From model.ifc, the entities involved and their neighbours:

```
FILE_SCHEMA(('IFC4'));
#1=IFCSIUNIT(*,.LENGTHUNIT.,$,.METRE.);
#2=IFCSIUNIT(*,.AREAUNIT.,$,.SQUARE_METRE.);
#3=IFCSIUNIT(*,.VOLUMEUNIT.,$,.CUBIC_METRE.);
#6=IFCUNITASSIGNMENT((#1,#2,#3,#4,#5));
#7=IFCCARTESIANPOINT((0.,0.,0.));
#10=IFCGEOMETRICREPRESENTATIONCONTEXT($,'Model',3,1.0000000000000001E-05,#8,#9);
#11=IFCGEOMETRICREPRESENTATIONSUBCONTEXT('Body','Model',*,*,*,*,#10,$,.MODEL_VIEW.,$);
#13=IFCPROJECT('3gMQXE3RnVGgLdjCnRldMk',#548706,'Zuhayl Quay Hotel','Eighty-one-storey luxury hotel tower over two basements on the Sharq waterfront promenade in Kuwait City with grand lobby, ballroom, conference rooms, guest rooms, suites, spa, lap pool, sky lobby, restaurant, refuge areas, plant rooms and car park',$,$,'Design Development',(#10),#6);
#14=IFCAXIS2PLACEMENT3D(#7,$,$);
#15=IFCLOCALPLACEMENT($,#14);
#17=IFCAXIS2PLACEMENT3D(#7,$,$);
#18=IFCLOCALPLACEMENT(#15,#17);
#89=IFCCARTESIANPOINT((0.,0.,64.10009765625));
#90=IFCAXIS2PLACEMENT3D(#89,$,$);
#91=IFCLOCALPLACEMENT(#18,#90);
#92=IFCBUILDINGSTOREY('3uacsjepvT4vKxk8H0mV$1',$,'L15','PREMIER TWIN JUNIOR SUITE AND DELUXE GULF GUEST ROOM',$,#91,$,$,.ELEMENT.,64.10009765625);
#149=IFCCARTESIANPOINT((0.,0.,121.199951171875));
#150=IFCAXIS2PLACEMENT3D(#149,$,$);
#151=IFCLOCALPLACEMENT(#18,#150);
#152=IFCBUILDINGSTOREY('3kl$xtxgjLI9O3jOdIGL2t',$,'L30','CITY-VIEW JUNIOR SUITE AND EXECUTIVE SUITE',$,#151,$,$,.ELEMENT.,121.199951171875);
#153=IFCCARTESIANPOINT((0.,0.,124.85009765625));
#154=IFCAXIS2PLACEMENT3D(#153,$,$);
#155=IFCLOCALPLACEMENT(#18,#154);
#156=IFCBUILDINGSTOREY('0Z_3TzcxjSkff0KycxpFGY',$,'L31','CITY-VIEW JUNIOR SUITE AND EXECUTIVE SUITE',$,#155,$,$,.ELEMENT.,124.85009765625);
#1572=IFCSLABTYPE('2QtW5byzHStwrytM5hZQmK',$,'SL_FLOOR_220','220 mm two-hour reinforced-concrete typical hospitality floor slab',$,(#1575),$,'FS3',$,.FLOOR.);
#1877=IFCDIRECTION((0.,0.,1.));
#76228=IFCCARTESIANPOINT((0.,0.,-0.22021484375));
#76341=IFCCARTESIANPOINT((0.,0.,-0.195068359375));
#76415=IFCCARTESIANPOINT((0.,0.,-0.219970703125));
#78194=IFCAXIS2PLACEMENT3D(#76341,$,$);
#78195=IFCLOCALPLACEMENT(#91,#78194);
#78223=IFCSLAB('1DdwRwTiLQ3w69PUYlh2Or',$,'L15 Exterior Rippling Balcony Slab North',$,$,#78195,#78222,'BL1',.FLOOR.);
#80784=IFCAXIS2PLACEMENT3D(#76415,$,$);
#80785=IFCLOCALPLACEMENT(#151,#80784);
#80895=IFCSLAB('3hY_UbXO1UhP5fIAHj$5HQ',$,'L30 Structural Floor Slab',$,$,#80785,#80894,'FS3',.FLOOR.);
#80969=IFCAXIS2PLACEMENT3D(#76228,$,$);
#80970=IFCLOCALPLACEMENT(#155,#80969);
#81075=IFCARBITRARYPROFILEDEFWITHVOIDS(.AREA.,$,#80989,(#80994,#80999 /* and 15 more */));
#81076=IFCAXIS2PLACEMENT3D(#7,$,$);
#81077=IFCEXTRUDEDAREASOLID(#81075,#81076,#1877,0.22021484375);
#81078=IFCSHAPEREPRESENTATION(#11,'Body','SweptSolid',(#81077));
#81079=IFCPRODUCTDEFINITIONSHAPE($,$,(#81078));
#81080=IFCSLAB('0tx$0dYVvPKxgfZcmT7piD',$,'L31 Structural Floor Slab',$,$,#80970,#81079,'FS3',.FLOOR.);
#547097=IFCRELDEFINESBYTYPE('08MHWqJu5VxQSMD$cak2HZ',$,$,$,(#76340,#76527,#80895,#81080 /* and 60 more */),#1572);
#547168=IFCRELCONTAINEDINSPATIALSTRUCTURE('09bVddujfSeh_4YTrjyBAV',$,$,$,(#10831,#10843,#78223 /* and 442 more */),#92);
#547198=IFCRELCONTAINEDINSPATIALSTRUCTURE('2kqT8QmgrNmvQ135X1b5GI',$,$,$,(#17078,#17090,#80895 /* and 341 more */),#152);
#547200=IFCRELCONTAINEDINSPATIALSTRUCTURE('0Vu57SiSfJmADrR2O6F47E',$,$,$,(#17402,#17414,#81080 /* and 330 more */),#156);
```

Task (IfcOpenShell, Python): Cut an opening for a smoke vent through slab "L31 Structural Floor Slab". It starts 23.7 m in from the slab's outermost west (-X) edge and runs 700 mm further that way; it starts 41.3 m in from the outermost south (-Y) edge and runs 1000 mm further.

```python
import numpy as np
import ifcopenshell
import ifcopenshell.api.feature
import ifcopenshell.api.geometry
import ifcopenshell.api.root
import ifcopenshell.geom
import ifcopenshell.util.placement
import ifcopenshell.util.representation
import ifcopenshell.util.shape
import ifcopenshell.util.unit

model = ifcopenshell.open("model.ifc")
unit_scale = ifcopenshell.util.unit.calculate_unit_scale(model)
settings = ifcopenshell.geom.settings()


def volume(element):
    """Net volume in cubic metres, openings subtracted."""
    shape = ifcopenshell.geom.create_shape(settings, element)
    return ifcopenshell.util.shape.get_volume(shape.geometry)


slab = model.by_id(81080)
before = volume(slab)

# Extent in the slab's own axes, in metres. The edges named are its -X and -Y sides.
slab_shape = ifcopenshell.geom.create_shape(settings, slab)
vertices = ifcopenshell.util.shape.get_vertices(slab_shape.geometry)
x_min, y_min, bottom = vertices.min(axis=0)
top = vertices[:, 2].max()

opening = ifcopenshell.api.root.create_entity(model, ifc_class="IfcOpeningElement", name="Smoke vent opening", predefined_type="OPENING")
context = ifcopenshell.util.representation.get_context(model, "Model", "Body", "MODEL_VIEW")
width, depth = 0.7, 1
outline = [(0.0, 0.0), (width, 0.0), (width, depth), (0.0, depth), (0.0, 0.0)]
# Overshoot both faces by 50 mm so the cut is clean.
shape = ifcopenshell.api.geometry.add_slab_representation(
    model, context=context, depth=top - bottom + 0.1, polyline=outline
)
ifcopenshell.api.geometry.assign_representation(model, product=opening, representation=shape)

matrix = ifcopenshell.util.placement.get_local_placement(slab.ObjectPlacement)
matrix[:, 3] = matrix @ np.append(np.array([x_min + 23.7, y_min + 41.3, bottom - 0.05]) / unit_scale, 1.0)
ifcopenshell.api.geometry.edit_object_placement(model, product=opening, matrix=matrix, is_si=False)
ifcopenshell.api.feature.add_feature(model, feature=opening, element=slab)

after = volume(slab)

print(f"slab volume {before:.3f} -> {after:.3f} m3")

model.write("model_edited.ifc")
```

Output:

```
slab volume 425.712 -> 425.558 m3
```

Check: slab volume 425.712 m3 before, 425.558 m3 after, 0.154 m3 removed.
